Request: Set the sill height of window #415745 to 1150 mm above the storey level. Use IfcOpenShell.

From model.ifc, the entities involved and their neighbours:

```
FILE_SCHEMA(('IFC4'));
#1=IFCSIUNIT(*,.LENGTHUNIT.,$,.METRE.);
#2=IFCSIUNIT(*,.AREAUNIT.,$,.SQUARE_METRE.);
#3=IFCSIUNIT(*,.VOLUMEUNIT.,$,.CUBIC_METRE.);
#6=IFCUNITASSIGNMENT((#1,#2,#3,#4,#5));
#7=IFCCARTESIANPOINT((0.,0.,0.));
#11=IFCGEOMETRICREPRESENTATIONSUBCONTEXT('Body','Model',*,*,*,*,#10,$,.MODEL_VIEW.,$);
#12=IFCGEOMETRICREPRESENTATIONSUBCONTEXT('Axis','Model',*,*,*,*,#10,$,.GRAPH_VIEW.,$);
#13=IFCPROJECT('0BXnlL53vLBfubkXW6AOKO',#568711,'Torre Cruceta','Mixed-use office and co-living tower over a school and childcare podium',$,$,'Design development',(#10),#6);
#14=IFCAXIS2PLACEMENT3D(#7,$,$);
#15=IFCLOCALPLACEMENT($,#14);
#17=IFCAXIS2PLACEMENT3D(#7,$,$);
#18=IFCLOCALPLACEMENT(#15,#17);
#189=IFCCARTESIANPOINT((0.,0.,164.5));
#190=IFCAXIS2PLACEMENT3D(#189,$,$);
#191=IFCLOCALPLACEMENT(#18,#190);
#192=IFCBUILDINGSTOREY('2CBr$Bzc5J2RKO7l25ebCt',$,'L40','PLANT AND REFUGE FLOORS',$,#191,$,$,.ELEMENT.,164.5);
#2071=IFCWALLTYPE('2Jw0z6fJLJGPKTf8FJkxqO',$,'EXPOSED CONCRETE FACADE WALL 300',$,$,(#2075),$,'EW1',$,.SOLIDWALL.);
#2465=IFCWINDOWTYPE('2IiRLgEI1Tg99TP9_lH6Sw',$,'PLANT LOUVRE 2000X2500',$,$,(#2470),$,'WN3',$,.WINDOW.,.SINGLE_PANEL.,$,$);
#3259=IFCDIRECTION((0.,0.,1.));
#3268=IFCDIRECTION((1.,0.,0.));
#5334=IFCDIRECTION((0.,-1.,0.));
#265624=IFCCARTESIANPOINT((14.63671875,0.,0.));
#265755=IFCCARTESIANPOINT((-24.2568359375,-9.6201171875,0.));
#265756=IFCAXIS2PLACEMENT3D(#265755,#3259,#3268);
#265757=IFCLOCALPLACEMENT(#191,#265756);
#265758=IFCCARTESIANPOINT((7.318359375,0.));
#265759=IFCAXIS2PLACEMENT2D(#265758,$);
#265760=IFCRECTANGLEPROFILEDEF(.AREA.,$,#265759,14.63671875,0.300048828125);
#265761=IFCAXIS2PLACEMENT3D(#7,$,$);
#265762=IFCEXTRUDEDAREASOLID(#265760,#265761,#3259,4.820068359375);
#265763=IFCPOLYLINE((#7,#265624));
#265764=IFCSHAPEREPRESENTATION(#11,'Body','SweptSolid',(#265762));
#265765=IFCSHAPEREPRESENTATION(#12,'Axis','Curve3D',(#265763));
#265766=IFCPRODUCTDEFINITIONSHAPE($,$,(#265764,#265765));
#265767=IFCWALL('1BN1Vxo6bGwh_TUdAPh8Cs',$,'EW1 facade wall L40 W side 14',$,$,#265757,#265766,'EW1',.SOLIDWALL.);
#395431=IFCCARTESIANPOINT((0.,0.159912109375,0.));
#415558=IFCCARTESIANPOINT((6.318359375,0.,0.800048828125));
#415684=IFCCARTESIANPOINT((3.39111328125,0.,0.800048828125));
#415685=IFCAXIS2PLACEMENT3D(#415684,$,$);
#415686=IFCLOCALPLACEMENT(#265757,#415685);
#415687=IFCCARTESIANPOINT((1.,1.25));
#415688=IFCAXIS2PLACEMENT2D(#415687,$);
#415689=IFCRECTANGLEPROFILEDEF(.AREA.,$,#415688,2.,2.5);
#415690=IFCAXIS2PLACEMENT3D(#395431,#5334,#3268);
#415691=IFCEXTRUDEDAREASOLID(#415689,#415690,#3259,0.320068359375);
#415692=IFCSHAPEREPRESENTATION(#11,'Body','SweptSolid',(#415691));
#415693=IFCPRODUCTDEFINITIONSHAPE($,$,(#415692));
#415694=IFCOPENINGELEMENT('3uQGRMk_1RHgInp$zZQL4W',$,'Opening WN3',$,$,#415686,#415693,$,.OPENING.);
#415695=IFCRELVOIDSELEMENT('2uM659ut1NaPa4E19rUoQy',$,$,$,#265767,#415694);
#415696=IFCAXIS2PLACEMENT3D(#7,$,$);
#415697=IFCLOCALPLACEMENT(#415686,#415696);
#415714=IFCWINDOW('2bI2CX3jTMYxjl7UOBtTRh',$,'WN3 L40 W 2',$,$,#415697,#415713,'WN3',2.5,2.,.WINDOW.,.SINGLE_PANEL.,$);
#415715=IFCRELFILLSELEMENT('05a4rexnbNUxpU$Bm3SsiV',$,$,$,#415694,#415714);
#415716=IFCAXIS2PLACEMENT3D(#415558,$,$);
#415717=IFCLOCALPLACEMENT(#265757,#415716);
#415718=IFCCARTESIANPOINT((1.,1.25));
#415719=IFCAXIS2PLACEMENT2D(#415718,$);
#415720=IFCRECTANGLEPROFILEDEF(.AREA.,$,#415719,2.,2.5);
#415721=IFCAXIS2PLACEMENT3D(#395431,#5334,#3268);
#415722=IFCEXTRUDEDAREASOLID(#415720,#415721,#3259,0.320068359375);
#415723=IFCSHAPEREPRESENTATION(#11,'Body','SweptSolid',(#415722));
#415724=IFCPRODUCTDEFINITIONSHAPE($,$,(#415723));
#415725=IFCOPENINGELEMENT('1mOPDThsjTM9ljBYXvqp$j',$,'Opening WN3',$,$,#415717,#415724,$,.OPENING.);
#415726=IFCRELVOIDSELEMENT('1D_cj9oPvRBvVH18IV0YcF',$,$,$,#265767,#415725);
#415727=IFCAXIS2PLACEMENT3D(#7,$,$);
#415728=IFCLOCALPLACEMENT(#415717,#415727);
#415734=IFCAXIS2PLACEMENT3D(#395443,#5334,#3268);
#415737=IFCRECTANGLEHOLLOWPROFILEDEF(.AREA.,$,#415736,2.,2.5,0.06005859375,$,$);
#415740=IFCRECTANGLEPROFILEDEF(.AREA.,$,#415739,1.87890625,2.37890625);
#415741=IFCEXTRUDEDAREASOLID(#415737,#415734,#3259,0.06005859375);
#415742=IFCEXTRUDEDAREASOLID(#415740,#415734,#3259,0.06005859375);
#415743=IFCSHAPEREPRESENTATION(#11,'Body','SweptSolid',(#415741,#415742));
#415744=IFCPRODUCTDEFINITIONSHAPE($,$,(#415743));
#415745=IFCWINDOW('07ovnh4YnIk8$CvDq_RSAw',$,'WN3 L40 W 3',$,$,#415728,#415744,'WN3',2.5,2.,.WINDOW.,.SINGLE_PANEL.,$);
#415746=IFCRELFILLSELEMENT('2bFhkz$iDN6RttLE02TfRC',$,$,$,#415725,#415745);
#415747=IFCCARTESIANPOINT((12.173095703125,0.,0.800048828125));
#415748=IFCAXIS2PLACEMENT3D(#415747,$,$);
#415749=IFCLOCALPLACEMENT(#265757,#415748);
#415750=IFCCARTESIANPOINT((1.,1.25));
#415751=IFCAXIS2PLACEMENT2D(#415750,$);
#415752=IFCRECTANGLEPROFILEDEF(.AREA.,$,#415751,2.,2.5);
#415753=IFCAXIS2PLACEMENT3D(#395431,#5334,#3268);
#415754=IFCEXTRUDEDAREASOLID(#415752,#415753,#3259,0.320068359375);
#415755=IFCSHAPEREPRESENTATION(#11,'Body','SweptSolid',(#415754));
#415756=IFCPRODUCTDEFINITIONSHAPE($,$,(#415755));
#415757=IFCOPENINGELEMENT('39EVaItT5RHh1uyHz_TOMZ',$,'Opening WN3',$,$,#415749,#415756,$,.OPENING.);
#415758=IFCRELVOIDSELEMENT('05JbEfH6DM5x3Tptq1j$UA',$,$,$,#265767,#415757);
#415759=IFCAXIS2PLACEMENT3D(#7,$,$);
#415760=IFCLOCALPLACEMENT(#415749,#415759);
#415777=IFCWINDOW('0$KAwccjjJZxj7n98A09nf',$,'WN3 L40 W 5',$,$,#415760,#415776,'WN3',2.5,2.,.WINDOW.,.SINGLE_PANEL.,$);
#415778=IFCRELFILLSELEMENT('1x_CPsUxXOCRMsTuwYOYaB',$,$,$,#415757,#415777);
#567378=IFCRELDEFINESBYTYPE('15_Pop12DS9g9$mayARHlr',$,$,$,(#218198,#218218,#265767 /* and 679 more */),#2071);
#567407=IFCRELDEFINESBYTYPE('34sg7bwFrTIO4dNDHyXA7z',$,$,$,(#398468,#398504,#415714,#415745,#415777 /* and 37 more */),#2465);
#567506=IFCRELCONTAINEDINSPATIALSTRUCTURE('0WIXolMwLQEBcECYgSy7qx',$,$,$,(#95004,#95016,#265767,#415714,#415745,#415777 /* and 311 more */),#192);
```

```python
import numpy as np
import ifcopenshell
import ifcopenshell.api.geometry
import ifcopenshell.geom
import ifcopenshell.util.element
import ifcopenshell.util.placement
import ifcopenshell.util.shape
import ifcopenshell.util.unit

model = ifcopenshell.open("model.ifc")
unit_scale = ifcopenshell.util.unit.calculate_unit_scale(model)

window = model.by_id(415745)
opening = window.FillsVoids[0].RelatingOpeningElement
storey = ifcopenshell.util.element.get_container(window, ifc_class="IfcBuildingStorey")
level = ifcopenshell.util.placement.get_local_placement(storey.ObjectPlacement)[2, 3]

# The opening's origin need not be at the sill, so measure its lowest point.
shape = ifcopenshell.geom.create_shape(ifcopenshell.geom.settings(), opening)
bottom = ifcopenshell.util.shape.get_shape_bottom_elevation(shape, shape.geometry) / unit_scale
dz = level + 1.15 / unit_scale - bottom

shift = np.array([0.0, 0.0, dz])
# The window is placed relative to its opening, so it follows when the opening moves.
matrix = ifcopenshell.util.placement.get_local_placement(opening.ObjectPlacement)
matrix[:3, 3] += shift
ifcopenshell.api.geometry.edit_object_placement(
    model, product=opening, matrix=matrix, is_si=False, should_transform_children=True
)

print(f"moved by {dz * unit_scale:+.3f} m")

model.write("model-out.ifc")
```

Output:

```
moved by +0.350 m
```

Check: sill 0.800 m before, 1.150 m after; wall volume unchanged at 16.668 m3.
